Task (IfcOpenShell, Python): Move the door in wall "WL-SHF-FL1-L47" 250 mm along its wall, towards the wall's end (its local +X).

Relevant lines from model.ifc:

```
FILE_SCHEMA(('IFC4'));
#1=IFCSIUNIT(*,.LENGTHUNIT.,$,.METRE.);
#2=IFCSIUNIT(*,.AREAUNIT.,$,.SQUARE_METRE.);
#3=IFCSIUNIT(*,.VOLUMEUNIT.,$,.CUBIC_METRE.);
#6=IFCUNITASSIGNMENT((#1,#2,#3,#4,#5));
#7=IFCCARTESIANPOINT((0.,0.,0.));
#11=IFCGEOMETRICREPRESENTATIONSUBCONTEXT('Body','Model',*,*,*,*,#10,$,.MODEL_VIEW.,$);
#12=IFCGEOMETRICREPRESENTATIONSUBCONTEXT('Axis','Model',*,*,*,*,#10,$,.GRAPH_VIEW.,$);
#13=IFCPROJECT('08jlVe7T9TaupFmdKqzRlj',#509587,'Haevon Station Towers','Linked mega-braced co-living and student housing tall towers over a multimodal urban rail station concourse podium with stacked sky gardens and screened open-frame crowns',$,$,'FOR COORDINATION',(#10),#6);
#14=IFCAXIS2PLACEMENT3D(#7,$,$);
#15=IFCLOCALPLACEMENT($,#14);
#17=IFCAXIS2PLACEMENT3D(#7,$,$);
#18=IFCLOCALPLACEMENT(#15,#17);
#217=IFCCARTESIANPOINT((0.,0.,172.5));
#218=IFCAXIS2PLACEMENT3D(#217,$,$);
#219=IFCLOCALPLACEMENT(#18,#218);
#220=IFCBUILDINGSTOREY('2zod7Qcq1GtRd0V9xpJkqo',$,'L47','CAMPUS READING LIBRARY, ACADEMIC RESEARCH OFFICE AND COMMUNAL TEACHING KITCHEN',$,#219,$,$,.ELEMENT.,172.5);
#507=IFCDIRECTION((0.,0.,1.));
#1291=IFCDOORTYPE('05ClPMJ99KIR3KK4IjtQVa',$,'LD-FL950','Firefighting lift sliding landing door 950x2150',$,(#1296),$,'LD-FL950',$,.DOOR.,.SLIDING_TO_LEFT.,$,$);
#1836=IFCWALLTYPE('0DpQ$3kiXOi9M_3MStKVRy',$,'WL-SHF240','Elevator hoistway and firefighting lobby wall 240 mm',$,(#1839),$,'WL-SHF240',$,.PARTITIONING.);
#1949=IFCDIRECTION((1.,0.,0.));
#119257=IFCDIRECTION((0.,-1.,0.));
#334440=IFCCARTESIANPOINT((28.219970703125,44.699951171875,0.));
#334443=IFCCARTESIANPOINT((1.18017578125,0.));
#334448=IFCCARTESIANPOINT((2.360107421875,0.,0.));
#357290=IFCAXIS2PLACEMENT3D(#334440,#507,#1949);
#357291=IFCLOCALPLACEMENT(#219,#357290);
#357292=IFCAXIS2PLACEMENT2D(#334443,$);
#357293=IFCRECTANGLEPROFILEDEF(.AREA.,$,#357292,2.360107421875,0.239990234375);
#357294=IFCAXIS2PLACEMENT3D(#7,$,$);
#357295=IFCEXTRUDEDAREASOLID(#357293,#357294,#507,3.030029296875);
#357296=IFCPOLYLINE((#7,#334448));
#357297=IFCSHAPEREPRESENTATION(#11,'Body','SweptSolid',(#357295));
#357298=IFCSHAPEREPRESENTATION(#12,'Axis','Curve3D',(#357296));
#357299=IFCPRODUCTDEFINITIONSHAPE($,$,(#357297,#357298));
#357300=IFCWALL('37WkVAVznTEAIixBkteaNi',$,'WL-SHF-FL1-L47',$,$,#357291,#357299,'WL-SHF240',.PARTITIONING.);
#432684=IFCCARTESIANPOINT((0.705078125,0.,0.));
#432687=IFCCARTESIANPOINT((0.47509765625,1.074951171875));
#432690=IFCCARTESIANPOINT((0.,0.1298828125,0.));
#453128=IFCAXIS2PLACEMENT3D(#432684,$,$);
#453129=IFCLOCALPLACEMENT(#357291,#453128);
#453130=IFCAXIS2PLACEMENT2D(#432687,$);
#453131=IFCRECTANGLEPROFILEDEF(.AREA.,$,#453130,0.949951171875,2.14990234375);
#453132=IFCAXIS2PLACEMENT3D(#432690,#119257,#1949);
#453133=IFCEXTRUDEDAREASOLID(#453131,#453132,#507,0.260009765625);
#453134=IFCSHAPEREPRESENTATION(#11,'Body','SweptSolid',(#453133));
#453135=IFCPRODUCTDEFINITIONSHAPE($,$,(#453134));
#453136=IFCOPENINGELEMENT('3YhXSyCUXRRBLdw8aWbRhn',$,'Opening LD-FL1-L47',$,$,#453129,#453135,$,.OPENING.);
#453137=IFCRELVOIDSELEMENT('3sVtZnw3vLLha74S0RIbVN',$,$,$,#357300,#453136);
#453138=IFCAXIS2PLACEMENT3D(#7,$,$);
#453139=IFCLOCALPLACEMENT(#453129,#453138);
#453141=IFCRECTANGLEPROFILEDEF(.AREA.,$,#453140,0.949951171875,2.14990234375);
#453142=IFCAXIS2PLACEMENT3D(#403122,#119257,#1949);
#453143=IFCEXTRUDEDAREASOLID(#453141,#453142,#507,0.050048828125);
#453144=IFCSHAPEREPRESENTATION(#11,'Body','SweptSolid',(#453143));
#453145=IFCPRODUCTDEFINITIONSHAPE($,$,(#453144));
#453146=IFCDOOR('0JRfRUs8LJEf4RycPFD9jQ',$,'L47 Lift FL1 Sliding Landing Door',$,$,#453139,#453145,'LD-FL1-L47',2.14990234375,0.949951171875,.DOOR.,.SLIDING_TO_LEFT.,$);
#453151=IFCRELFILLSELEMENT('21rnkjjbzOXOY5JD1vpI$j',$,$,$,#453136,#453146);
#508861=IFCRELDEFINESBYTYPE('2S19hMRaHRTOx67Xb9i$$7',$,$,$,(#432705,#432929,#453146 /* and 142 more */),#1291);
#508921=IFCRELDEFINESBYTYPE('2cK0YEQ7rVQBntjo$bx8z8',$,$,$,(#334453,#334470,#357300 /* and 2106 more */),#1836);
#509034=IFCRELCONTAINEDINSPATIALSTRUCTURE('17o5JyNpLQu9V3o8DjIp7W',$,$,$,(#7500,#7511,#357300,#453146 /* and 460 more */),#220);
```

```python
import ifcopenshell
import ifcopenshell.api.geometry
import ifcopenshell.util.placement

model = ifcopenshell.open("model.ifc")

door = model.by_guid("0JRfRUs8LJEf4RycPFD9jQ")
opening = door.FillsVoids[0].RelatingOpeningElement
wall = opening.VoidsElements[0].RelatingBuildingElement

wall_matrix = ifcopenshell.util.placement.get_local_placement(wall.ObjectPlacement)
shift = wall_matrix[:3, 0] * 0.25
before = ifcopenshell.util.placement.get_local_placement(door.ObjectPlacement)[:3, 3].copy()

# The door is placed relative to its opening, so it follows when the opening moves.
matrix = ifcopenshell.util.placement.get_local_placement(opening.ObjectPlacement)
matrix[:3, 3] += shift
ifcopenshell.api.geometry.edit_object_placement(
    model, product=opening, matrix=matrix, is_si=False, should_transform_children=True
)

after = ifcopenshell.util.placement.get_local_placement(door.ObjectPlacement)[:3, 3]
print("door moved by", (after - before).round(3) + 0.0)

model.write("model_updated.ifc")
```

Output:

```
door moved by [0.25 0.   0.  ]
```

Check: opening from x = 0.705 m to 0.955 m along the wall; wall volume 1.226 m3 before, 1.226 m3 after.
